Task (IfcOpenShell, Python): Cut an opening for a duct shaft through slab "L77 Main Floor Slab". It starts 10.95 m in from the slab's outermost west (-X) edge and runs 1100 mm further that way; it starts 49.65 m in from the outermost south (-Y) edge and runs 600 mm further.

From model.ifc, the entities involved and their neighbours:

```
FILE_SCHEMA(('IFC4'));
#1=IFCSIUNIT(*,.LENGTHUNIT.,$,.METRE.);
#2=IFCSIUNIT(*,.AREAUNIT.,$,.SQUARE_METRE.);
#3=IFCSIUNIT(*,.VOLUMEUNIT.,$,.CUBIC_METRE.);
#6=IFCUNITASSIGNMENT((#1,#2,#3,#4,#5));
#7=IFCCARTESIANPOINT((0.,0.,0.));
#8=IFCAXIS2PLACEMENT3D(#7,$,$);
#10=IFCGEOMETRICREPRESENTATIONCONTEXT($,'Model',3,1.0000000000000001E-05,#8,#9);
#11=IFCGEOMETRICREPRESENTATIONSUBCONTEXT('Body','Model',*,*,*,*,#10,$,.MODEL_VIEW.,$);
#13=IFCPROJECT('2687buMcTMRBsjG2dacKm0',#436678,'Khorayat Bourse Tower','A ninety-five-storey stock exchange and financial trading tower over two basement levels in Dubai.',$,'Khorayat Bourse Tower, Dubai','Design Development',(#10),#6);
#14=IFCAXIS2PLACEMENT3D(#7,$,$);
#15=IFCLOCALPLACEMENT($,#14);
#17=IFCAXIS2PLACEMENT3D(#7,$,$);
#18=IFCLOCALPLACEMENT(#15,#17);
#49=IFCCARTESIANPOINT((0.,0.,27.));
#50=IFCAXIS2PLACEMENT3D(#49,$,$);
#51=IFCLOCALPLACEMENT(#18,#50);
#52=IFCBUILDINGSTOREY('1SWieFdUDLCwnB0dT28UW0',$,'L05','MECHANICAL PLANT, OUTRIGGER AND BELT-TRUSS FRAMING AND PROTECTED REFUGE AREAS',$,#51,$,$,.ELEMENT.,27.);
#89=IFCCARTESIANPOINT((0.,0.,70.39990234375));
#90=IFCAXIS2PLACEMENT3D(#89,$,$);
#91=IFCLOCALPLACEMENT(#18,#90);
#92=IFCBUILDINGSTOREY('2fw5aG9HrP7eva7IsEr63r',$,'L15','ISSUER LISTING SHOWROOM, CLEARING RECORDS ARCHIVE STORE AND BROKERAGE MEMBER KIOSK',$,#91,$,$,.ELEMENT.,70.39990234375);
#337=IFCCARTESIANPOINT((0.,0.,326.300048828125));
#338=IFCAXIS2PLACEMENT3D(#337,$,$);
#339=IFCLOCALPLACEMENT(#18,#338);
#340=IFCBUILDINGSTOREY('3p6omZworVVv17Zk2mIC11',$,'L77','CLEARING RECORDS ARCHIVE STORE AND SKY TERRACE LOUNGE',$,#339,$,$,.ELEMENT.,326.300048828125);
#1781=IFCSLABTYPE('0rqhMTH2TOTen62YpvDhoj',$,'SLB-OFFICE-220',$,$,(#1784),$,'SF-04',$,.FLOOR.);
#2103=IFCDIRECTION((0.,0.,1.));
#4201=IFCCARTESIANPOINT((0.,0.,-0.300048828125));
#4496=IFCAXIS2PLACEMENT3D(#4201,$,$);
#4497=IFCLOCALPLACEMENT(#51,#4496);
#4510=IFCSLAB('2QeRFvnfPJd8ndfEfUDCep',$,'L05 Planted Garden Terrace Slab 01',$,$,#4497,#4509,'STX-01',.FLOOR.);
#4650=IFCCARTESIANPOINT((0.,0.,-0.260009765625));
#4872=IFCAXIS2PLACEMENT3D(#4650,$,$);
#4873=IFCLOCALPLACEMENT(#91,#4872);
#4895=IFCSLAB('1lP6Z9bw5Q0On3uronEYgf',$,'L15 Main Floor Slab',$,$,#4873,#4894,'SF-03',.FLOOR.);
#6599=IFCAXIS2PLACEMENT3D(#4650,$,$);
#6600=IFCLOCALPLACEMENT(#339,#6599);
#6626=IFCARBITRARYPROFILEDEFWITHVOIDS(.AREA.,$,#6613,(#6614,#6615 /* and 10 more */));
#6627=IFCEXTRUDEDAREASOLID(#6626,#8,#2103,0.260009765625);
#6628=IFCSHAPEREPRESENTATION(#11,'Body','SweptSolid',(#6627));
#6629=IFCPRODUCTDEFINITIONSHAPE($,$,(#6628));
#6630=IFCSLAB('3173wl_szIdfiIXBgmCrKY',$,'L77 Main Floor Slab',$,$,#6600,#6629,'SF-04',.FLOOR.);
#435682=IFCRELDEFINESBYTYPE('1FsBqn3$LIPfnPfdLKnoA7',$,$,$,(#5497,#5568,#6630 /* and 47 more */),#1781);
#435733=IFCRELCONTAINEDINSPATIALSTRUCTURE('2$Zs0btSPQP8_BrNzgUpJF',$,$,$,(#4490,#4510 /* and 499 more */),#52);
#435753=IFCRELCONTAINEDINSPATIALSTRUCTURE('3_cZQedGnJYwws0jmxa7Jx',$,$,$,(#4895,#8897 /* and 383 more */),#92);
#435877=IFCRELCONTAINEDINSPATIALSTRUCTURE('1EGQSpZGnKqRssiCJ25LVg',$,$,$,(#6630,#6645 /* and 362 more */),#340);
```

```python
import numpy as np
import ifcopenshell
import ifcopenshell.api.feature
import ifcopenshell.api.geometry
import ifcopenshell.api.root
import ifcopenshell.geom
import ifcopenshell.util.placement
import ifcopenshell.util.representation
import ifcopenshell.util.shape
import ifcopenshell.util.unit

model = ifcopenshell.open("model.ifc")
unit_scale = ifcopenshell.util.unit.calculate_unit_scale(model)
settings = ifcopenshell.geom.settings()


def volume(element):
    """Net volume in cubic metres, openings subtracted."""
    shape = ifcopenshell.geom.create_shape(settings, element)
    return ifcopenshell.util.shape.get_volume(shape.geometry)


slab = model.by_guid("3173wl_szIdfiIXBgmCrKY")
before = volume(slab)

# Extent in the slab's own axes, in metres. The edges named are its -X and -Y sides.
slab_shape = ifcopenshell.geom.create_shape(settings, slab)
vertices = ifcopenshell.util.shape.get_vertices(slab_shape.geometry)
x_min, y_min, bottom = vertices.min(axis=0)
top = vertices[:, 2].max()

opening = ifcopenshell.api.root.create_entity(model, ifc_class="IfcOpeningElement", name="Duct shaft opening", predefined_type="OPENING")
context = ifcopenshell.util.representation.get_context(model, "Model", "Body", "MODEL_VIEW")
width, depth = 1.1, 0.6
outline = [(0.0, 0.0), (width, 0.0), (width, depth), (0.0, depth), (0.0, 0.0)]
# Overshoot both faces by 50 mm so the cut is clean.
shape = ifcopenshell.api.geometry.add_slab_representation(
    model, context=context, depth=top - bottom + 0.1, polyline=outline
)
ifcopenshell.api.geometry.assign_representation(model, product=opening, representation=shape)

matrix = ifcopenshell.util.placement.get_local_placement(slab.ObjectPlacement)
matrix[:, 3] = matrix @ np.append(np.array([x_min + 10.95, y_min + 49.65, bottom - 0.05]) / unit_scale, 1.0)
ifcopenshell.api.geometry.edit_object_placement(model, product=opening, matrix=matrix, is_si=False)
ifcopenshell.api.feature.add_feature(model, feature=opening, element=slab)

after = volume(slab)

print(f"slab volume {before:.3f} -> {after:.3f} m3")

model.write("model-out.ifc")
```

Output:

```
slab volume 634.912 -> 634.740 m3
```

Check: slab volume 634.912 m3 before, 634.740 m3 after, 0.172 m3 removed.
